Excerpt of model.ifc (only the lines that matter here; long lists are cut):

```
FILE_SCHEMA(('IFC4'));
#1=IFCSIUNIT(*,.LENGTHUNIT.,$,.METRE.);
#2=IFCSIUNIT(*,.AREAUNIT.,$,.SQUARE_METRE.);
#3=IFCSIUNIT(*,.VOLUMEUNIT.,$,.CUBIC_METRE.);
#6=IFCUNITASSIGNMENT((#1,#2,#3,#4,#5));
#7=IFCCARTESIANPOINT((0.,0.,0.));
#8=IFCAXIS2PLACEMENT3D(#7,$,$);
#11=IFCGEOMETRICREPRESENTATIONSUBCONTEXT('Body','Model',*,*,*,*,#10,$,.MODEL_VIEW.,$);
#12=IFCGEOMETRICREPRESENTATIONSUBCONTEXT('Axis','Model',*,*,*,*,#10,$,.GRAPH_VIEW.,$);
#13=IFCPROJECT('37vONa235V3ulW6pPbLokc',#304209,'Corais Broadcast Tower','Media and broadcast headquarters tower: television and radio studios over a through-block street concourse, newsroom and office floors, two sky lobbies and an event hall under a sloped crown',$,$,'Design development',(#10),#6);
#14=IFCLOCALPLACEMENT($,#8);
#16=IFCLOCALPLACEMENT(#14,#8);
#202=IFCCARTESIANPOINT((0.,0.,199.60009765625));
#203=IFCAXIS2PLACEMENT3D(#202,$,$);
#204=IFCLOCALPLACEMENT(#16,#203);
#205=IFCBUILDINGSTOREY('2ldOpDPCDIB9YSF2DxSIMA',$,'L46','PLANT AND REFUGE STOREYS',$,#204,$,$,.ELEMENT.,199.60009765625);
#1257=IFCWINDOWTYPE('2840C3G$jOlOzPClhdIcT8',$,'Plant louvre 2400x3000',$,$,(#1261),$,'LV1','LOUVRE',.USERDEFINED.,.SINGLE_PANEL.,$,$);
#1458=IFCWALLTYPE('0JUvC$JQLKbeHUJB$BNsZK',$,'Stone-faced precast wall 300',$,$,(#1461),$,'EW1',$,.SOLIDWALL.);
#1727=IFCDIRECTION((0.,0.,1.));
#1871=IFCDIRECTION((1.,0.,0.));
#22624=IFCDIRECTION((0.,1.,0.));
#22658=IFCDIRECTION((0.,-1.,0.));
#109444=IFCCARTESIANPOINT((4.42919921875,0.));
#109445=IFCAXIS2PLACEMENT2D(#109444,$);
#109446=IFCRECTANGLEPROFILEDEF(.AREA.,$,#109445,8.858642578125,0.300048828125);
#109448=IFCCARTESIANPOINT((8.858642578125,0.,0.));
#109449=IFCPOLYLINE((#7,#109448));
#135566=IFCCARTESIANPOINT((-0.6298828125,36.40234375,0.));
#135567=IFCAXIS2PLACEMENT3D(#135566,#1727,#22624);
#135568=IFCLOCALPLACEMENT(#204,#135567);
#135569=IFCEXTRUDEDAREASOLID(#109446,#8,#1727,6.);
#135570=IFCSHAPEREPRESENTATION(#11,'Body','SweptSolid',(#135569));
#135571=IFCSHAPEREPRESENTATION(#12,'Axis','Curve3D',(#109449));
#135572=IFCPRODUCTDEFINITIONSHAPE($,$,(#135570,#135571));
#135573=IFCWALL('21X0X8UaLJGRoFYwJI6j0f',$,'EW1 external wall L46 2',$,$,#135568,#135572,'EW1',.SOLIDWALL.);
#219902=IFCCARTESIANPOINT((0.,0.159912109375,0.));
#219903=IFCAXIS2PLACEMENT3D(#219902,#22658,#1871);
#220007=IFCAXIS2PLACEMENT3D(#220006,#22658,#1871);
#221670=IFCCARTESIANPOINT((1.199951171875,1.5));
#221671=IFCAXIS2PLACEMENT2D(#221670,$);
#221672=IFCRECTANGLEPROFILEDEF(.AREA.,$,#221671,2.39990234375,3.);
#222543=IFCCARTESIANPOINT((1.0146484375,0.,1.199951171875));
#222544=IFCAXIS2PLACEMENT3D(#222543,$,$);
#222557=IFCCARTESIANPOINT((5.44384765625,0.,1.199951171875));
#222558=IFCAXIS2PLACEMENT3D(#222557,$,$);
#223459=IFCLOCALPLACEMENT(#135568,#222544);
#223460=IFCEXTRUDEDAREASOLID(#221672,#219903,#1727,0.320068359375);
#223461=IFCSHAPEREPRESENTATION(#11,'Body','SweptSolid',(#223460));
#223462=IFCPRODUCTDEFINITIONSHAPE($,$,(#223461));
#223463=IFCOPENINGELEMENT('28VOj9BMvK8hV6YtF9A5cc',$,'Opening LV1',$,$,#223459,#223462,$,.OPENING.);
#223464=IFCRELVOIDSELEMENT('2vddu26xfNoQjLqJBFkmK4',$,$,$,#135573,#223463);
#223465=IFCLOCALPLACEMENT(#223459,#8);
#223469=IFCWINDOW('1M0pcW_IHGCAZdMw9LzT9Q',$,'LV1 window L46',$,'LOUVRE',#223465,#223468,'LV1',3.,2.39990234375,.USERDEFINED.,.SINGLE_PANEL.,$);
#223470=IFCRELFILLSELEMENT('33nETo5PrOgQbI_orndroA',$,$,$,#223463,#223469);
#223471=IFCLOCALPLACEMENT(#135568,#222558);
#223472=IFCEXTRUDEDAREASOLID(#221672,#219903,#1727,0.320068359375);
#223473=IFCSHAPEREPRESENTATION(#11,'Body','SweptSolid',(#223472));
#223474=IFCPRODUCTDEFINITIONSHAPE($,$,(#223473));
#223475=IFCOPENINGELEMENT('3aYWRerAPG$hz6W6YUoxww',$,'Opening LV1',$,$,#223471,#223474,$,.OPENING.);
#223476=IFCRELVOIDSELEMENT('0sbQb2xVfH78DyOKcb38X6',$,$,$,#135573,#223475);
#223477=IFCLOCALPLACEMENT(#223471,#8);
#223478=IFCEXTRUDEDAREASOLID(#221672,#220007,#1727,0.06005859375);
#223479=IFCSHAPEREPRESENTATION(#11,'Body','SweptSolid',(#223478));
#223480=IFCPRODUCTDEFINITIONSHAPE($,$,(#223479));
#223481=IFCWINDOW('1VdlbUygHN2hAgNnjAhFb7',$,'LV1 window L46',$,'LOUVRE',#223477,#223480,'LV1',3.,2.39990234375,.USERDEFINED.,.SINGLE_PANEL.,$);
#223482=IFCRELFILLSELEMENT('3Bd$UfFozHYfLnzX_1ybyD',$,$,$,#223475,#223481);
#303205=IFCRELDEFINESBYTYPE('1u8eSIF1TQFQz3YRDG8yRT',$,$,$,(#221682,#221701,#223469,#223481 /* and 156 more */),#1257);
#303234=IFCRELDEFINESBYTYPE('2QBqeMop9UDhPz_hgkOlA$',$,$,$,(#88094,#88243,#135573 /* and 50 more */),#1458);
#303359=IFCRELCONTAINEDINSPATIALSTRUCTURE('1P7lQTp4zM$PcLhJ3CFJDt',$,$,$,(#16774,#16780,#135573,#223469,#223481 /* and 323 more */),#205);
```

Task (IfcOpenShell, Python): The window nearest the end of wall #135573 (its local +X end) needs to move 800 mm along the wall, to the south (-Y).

```python
import ifcopenshell
import ifcopenshell.api.geometry
import ifcopenshell.util.placement
import ifcopenshell.util.unit

model = ifcopenshell.open("model.ifc")
unit_scale = ifcopenshell.util.unit.calculate_unit_scale(model)

window = model.by_guid("1VdlbUygHN2hAgNnjAhFb7")
opening = window.FillsVoids[0].RelatingOpeningElement
wall = opening.VoidsElements[0].RelatingBuildingElement

wall_matrix = ifcopenshell.util.placement.get_local_placement(wall.ObjectPlacement)
shift = wall_matrix[:3, 0] * -0.8 / unit_scale
before = ifcopenshell.util.placement.get_local_placement(window.ObjectPlacement)[:3, 3].copy()

# The window is placed relative to its opening, so it follows when the opening moves.
matrix = ifcopenshell.util.placement.get_local_placement(opening.ObjectPlacement)
matrix[:3, 3] += shift
ifcopenshell.api.geometry.edit_object_placement(
    model, product=opening, matrix=matrix, is_si=False, should_transform_children=True
)

after = ifcopenshell.util.placement.get_local_placement(window.ObjectPlacement)[:3, 3]
print("window moved by", (after - before).round(3) + 0.0)

model.write("model-out.ifc")
```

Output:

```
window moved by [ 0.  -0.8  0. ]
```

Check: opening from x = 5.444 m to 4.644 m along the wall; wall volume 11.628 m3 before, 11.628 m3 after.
